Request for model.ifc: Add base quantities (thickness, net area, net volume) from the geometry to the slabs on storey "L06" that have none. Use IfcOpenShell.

First a look at what the model holds.

```python
import ifcopenshell
import ifcopenshell.util.element
import ifcopenshell.util.unit

model = ifcopenshell.open("model.ifc")
print(model.schema)
for unit_type in ("LENGTHUNIT", "AREAUNIT", "VOLUMEUNIT"):
    print(unit_type, ifcopenshell.util.unit.calculate_unit_scale(model, unit_type))
storey = next(s for s in model.by_type("IfcBuildingStorey") if s.Name == "L06")
slabs = [e for e in ifcopenshell.util.element.get_decomposition(storey) if e.is_a("IfcSlab")]
for e in sorted(slabs, key=lambda e: e.id()):
    print(e.id(), e.is_a(), e.Name, list(ifcopenshell.util.element.get_psets(e, qtos_only=True)), sep=" | ")
```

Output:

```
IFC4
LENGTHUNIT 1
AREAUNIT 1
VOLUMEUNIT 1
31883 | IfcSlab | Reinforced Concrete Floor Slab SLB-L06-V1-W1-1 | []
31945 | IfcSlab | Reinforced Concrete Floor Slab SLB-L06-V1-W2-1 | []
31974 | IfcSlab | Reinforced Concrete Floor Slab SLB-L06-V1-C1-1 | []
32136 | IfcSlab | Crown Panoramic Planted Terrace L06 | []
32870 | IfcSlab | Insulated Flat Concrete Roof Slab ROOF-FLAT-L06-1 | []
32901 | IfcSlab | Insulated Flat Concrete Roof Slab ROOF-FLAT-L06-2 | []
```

```python
import ifcopenshell
import ifcopenshell.api.pset
import ifcopenshell.geom
import ifcopenshell.util.element
import ifcopenshell.util.shape
import ifcopenshell.util.unit

model = ifcopenshell.open("model.ifc")
unit_scale = ifcopenshell.util.unit.calculate_unit_scale(model)
area_scale = ifcopenshell.util.unit.calculate_unit_scale(model, "AREAUNIT")
volume_scale = ifcopenshell.util.unit.calculate_unit_scale(model, "VOLUMEUNIT")
settings = ifcopenshell.geom.settings()

storey = next(s for s in model.by_type("IfcBuildingStorey") if s.Name == "L06")
slabs = [e for e in ifcopenshell.util.element.get_decomposition(storey) if e.is_a("IfcSlab")]

for e in sorted(slabs, key=lambda e: e.id()):
    if ifcopenshell.util.element.get_psets(e, qtos_only=True, should_inherit=False):
        continue
    # Geometry comes back in metres, in the element's own axes.
    shape = ifcopenshell.geom.create_shape(settings, e)
    values = {
        "Width": ifcopenshell.util.shape.get_z(shape.geometry) / unit_scale,
        "NetArea": ifcopenshell.util.shape.get_footprint_area(shape.geometry) / area_scale,
        "NetVolume": ifcopenshell.util.shape.get_volume(shape.geometry) / volume_scale,
    }
    qto = ifcopenshell.api.pset.add_qto(model, product=e, name="Qto_SlabBaseQuantities")
    ifcopenshell.api.pset.edit_qto(model, qto=qto, properties=values)
    print(e.id(), {k: round(v, 3) for k, v in values.items()})

model.write("model_rev.ifc")
```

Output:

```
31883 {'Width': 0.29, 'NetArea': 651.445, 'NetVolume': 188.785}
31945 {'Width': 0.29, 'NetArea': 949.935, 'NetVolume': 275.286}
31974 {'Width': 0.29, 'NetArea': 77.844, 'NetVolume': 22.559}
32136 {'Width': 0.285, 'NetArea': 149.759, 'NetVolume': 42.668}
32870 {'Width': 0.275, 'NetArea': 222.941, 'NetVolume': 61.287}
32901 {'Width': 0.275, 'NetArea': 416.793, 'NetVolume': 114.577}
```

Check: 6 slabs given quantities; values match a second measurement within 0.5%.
